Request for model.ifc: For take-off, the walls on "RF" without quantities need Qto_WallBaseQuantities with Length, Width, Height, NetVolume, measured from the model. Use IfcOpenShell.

First a look at what the model holds.

```python
import ifcopenshell
import ifcopenshell.util.element
import ifcopenshell.util.unit

model = ifcopenshell.open("model.ifc")
print(model.schema)
for unit_type in ("LENGTHUNIT", "AREAUNIT", "VOLUMEUNIT"):
    print(unit_type, ifcopenshell.util.unit.calculate_unit_scale(model, unit_type))
storey = next(s for s in model.by_type("IfcBuildingStorey") if s.Name == "RF")
walls = [e for e in ifcopenshell.util.element.get_decomposition(storey) if e.is_a("IfcWall")]
for e in sorted(walls, key=lambda e: e.id()):
    print(e.id(), e.is_a(), e.Name, list(ifcopenshell.util.element.get_psets(e, qtos_only=True)), sep=" | ")
```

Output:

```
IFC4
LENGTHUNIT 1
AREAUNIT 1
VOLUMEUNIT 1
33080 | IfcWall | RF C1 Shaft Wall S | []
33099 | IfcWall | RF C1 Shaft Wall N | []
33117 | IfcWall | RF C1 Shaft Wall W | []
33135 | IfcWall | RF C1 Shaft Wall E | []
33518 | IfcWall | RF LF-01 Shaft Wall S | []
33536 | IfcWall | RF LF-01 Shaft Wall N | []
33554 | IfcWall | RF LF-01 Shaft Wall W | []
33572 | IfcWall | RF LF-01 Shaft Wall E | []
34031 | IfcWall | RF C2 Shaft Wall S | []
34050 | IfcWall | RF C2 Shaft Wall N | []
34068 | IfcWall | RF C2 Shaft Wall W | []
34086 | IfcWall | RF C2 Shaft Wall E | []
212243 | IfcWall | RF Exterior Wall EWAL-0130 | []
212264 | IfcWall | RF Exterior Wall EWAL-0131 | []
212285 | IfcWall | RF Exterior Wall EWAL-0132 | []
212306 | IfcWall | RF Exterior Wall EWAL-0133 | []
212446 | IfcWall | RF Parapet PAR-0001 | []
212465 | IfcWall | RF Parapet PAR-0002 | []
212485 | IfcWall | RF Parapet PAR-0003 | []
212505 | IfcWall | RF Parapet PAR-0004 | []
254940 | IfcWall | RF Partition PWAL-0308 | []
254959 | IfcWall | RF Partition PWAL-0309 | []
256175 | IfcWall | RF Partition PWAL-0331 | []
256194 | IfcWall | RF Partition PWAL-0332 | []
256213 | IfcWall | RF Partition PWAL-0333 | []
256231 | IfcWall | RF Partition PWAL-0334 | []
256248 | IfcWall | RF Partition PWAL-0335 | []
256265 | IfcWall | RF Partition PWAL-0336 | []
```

```python
import ifcopenshell
import ifcopenshell.api.pset
import ifcopenshell.geom
import ifcopenshell.util.element
import ifcopenshell.util.shape
import ifcopenshell.util.unit

model = ifcopenshell.open("model.ifc")
unit_scale = ifcopenshell.util.unit.calculate_unit_scale(model)
volume_scale = ifcopenshell.util.unit.calculate_unit_scale(model, "VOLUMEUNIT")
settings = ifcopenshell.geom.settings()

storey = next(s for s in model.by_type("IfcBuildingStorey") if s.Name == "RF")
walls = [e for e in ifcopenshell.util.element.get_decomposition(storey) if e.is_a("IfcWall")]

for e in sorted(walls, key=lambda e: e.id()):
    if ifcopenshell.util.element.get_psets(e, qtos_only=True, should_inherit=False):
        continue
    # Geometry comes back in metres, in the element's own axes.
    shape = ifcopenshell.geom.create_shape(settings, e)
    values = {
        "Length": ifcopenshell.util.shape.get_x(shape.geometry) / unit_scale,
        "Width": ifcopenshell.util.shape.get_y(shape.geometry) / unit_scale,
        "Height": ifcopenshell.util.shape.get_z(shape.geometry) / unit_scale,
        "NetVolume": ifcopenshell.util.shape.get_volume(shape.geometry) / volume_scale,
    }
    qto = ifcopenshell.api.pset.add_qto(model, product=e, name="Qto_WallBaseQuantities")
    ifcopenshell.api.pset.edit_qto(model, qto=qto, properties=values)
    print(e.id(), {k: round(v, 3) for k, v in values.items()})

model.write("model_updated.ifc")
```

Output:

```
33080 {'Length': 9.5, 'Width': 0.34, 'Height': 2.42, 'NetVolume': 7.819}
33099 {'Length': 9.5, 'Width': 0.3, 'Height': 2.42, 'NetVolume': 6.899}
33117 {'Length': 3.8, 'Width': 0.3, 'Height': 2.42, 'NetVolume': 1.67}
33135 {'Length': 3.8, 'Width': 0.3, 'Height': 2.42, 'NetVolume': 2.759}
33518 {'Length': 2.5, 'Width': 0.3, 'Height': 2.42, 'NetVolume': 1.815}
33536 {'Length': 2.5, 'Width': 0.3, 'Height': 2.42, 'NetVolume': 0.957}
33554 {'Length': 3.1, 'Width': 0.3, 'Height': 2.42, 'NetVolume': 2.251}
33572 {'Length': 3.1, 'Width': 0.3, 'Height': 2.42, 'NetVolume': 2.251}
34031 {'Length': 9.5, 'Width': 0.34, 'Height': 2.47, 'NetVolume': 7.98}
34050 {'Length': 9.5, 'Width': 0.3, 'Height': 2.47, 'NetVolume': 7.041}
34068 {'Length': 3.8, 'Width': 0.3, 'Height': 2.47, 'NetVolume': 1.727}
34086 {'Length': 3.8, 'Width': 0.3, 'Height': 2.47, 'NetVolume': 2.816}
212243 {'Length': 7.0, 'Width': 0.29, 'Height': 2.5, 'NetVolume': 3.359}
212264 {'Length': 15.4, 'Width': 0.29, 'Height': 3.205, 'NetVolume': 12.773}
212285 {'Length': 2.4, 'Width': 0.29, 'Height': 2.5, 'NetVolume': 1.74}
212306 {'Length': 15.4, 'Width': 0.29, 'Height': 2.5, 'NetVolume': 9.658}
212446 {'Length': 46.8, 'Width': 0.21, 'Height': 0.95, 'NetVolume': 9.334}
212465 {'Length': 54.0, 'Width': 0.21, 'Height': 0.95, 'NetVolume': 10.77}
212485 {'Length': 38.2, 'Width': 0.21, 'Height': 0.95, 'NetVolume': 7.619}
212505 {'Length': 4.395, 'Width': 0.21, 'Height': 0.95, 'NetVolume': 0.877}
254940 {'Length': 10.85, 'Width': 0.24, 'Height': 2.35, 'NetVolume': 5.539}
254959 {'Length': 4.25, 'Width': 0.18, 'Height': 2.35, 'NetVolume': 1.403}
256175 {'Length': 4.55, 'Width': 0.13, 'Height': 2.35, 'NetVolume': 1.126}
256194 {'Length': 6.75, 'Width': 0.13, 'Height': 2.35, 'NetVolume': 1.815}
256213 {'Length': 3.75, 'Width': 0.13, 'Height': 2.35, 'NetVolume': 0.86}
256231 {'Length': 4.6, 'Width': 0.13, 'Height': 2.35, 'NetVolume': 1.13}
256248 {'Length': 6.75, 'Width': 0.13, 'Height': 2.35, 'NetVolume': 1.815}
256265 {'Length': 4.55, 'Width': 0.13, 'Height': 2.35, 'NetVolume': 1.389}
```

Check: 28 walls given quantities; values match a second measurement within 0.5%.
